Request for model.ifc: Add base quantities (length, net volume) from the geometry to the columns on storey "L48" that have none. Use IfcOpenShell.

First a look at what the model holds.

```python
import ifcopenshell
import ifcopenshell.util.element
import ifcopenshell.util.unit

model = ifcopenshell.open("model.ifc")
print(model.schema)
for unit_type in ("LENGTHUNIT", "AREAUNIT", "VOLUMEUNIT"):
    print(unit_type, ifcopenshell.util.unit.calculate_unit_scale(model, unit_type))
storey = next(s for s in model.by_type("IfcBuildingStorey") if s.Name == "L48")
columns = [e for e in ifcopenshell.util.element.get_decomposition(storey) if e.is_a("IfcColumn")]
for e in sorted(columns, key=lambda e: e.id()):
    print(e.id(), e.is_a(), e.Name, list(ifcopenshell.util.element.get_psets(e, qtos_only=True)), sep=" | ")
```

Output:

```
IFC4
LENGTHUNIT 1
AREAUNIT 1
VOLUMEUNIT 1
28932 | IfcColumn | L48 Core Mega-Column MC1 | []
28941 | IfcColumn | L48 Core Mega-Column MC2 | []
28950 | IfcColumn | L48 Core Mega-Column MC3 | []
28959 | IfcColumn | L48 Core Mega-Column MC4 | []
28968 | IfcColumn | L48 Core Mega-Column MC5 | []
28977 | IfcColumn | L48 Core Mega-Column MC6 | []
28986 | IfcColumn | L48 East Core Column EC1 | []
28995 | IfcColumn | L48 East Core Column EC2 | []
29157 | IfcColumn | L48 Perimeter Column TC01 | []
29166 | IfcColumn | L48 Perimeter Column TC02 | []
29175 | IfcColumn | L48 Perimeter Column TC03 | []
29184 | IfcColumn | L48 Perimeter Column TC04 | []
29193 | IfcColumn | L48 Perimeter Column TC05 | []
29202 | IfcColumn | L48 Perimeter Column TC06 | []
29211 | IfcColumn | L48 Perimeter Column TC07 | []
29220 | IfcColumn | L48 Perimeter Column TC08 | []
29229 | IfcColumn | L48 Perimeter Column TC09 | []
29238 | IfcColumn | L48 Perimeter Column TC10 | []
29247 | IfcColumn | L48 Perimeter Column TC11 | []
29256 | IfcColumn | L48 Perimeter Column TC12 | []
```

```python
import ifcopenshell
import ifcopenshell.api.pset
import ifcopenshell.geom
import ifcopenshell.util.element
import ifcopenshell.util.shape
import ifcopenshell.util.unit

model = ifcopenshell.open("model.ifc")
unit_scale = ifcopenshell.util.unit.calculate_unit_scale(model)
volume_scale = ifcopenshell.util.unit.calculate_unit_scale(model, "VOLUMEUNIT")
settings = ifcopenshell.geom.settings()

storey = next(s for s in model.by_type("IfcBuildingStorey") if s.Name == "L48")
columns = [e for e in ifcopenshell.util.element.get_decomposition(storey) if e.is_a("IfcColumn")]

for e in sorted(columns, key=lambda e: e.id()):
    if ifcopenshell.util.element.get_psets(e, qtos_only=True, should_inherit=False):
        continue
    # Geometry comes back in metres, in the element's own axes.
    shape = ifcopenshell.geom.create_shape(settings, e)
    values = {
        "Length": ifcopenshell.util.shape.get_z(shape.geometry) / unit_scale,
        "NetVolume": ifcopenshell.util.shape.get_volume(shape.geometry) / volume_scale,
    }
    qto = ifcopenshell.api.pset.add_qto(model, product=e, name="Qto_ColumnBaseQuantities")
    ifcopenshell.api.pset.edit_qto(model, qto=qto, properties=values)
    print(e.id(), {k: round(v, 3) for k, v in values.items()})

model.write("model_updated.ifc")
```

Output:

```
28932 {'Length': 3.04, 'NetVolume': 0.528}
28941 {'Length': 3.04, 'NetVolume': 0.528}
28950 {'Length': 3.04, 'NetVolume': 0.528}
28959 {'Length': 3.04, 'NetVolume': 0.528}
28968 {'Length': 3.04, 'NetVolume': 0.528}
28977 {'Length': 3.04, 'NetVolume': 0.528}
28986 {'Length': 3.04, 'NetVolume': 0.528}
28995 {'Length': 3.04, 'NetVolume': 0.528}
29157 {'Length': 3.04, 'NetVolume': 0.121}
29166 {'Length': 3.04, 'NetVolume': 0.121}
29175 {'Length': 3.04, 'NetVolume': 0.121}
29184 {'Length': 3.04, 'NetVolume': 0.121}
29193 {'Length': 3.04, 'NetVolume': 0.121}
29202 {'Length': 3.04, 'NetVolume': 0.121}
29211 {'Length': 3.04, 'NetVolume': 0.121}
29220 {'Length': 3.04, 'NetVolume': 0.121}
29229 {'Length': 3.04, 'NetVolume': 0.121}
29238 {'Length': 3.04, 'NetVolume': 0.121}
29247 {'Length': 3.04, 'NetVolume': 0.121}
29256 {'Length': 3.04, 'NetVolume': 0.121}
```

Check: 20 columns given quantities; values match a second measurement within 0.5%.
